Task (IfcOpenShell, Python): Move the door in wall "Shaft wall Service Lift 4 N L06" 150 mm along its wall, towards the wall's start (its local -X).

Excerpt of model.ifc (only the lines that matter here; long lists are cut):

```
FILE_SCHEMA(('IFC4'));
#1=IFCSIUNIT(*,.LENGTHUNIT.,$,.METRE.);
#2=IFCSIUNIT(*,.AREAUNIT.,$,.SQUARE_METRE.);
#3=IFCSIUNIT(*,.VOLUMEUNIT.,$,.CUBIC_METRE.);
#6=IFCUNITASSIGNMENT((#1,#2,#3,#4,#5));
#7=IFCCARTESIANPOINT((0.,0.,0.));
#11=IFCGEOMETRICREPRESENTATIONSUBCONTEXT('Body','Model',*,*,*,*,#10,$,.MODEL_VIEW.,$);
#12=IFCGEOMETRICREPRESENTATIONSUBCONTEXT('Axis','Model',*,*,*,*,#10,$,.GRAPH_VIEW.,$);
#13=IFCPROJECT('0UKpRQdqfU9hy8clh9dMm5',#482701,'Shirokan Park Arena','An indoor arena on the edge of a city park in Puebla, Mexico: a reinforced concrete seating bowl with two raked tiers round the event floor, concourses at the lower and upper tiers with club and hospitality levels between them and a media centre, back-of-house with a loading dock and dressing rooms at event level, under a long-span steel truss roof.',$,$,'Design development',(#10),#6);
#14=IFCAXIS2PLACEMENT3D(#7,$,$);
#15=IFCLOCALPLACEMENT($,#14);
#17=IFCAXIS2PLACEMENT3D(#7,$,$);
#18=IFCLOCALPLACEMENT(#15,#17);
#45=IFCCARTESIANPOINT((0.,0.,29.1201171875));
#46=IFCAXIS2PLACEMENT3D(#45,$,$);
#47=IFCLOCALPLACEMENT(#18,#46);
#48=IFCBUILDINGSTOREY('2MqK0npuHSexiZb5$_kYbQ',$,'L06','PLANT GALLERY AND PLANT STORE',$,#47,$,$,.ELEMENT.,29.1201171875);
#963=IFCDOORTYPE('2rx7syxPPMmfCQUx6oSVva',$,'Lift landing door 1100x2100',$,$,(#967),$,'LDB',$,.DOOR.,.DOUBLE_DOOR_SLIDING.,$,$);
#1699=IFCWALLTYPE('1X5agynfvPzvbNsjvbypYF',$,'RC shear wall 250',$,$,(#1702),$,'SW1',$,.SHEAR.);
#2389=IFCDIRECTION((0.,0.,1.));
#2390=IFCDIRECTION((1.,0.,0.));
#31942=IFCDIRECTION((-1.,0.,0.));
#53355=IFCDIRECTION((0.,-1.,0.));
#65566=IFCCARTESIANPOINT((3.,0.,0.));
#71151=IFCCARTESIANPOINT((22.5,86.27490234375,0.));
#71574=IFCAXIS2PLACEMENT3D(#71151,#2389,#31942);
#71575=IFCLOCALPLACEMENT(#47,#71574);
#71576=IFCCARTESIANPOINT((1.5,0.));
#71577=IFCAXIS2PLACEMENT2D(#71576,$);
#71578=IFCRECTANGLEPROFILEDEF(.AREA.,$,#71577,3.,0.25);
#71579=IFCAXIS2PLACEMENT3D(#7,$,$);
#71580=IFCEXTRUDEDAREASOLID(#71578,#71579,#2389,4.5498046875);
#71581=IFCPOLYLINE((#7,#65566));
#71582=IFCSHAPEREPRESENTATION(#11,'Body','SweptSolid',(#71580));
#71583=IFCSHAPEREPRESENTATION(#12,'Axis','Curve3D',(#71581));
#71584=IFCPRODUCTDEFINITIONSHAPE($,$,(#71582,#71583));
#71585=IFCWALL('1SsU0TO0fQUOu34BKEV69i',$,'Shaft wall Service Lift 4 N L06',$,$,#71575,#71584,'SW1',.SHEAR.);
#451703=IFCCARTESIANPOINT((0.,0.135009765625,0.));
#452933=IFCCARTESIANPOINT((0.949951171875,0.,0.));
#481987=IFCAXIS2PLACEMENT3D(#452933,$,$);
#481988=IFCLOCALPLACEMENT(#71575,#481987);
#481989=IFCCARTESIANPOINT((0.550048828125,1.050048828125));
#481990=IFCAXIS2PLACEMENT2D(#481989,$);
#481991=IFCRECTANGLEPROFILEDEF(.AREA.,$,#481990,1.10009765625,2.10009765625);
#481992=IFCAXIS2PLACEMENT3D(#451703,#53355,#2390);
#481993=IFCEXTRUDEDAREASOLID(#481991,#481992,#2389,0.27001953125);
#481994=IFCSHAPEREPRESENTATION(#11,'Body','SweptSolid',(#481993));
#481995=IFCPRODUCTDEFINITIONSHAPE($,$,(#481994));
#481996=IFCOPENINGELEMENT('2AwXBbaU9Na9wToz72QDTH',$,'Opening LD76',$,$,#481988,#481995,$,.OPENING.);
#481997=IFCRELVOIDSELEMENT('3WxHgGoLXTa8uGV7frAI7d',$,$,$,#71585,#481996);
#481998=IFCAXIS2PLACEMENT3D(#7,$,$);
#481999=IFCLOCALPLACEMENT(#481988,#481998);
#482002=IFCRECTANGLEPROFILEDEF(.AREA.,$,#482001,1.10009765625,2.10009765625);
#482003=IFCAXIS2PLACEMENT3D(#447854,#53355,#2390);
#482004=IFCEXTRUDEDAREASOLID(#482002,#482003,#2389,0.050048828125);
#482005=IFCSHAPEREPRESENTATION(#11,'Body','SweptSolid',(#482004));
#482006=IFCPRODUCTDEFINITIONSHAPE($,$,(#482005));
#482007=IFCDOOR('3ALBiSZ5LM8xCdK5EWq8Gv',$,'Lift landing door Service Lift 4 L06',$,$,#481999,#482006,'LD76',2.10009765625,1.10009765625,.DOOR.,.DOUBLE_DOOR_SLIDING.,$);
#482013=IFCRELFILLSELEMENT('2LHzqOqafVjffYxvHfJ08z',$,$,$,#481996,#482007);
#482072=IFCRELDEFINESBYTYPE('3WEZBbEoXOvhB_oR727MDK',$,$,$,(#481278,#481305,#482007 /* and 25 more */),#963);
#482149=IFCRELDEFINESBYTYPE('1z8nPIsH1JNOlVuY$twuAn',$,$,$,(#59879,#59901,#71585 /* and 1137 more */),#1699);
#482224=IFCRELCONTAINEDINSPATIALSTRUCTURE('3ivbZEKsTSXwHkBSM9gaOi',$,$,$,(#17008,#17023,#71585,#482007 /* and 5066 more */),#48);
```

```python
import ifcopenshell
import ifcopenshell.api.geometry
import ifcopenshell.util.placement
import ifcopenshell.util.unit

model = ifcopenshell.open("model.ifc")
unit_scale = ifcopenshell.util.unit.calculate_unit_scale(model)

door = model.by_guid("3ALBiSZ5LM8xCdK5EWq8Gv")
opening = door.FillsVoids[0].RelatingOpeningElement
wall = opening.VoidsElements[0].RelatingBuildingElement

wall_matrix = ifcopenshell.util.placement.get_local_placement(wall.ObjectPlacement)
shift = wall_matrix[:3, 0] * -0.15 / unit_scale
before = ifcopenshell.util.placement.get_local_placement(door.ObjectPlacement)[:3, 3].copy()

# The door is placed relative to its opening, so it follows when the opening moves.
matrix = ifcopenshell.util.placement.get_local_placement(opening.ObjectPlacement)
matrix[:3, 3] += shift
ifcopenshell.api.geometry.edit_object_placement(
    model, product=opening, matrix=matrix, is_si=False, should_transform_children=True
)

after = ifcopenshell.util.placement.get_local_placement(door.ObjectPlacement)[:3, 3]
print("door moved by", (after - before).round(3) + 0.0)

model.write("model_updated.ifc")
```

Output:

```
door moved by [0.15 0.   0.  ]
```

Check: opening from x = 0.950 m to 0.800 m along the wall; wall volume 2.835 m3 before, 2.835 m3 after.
